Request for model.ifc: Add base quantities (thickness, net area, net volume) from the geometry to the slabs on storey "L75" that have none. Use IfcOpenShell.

First a look at what the model holds.

```python
import ifcopenshell
import ifcopenshell.util.element
import ifcopenshell.util.unit

model = ifcopenshell.open("model.ifc")
print(model.schema)
for unit_type in ("LENGTHUNIT", "AREAUNIT", "VOLUMEUNIT"):
    print(unit_type, ifcopenshell.util.unit.calculate_unit_scale(model, unit_type))
storey = next(s for s in model.by_type("IfcBuildingStorey") if s.Name == "L75")
slabs = [e for e in ifcopenshell.util.element.get_decomposition(storey) if e.is_a("IfcSlab")]
for e in sorted(slabs, key=lambda e: e.id()):
    print(e.id(), e.is_a(), e.Name, list(ifcopenshell.util.element.get_psets(e, qtos_only=True)), sep=" | ")
```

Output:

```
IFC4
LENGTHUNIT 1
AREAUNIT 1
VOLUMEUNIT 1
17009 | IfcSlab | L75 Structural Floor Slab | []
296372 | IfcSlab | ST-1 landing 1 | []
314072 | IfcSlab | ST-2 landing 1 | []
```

```python
import ifcopenshell
import ifcopenshell.api.pset
import ifcopenshell.geom
import ifcopenshell.util.element
import ifcopenshell.util.shape
import ifcopenshell.util.unit

model = ifcopenshell.open("model.ifc")
unit_scale = ifcopenshell.util.unit.calculate_unit_scale(model)
area_scale = ifcopenshell.util.unit.calculate_unit_scale(model, "AREAUNIT")
volume_scale = ifcopenshell.util.unit.calculate_unit_scale(model, "VOLUMEUNIT")
settings = ifcopenshell.geom.settings()

storey = next(s for s in model.by_type("IfcBuildingStorey") if s.Name == "L75")
slabs = [e for e in ifcopenshell.util.element.get_decomposition(storey) if e.is_a("IfcSlab")]

for e in sorted(slabs, key=lambda e: e.id()):
    if ifcopenshell.util.element.get_psets(e, qtos_only=True, should_inherit=False):
        continue
    # Geometry comes back in metres, in the element's own axes.
    shape = ifcopenshell.geom.create_shape(settings, e)
    values = {
        "Width": ifcopenshell.util.shape.get_z(shape.geometry) / unit_scale,
        "NetArea": ifcopenshell.util.shape.get_footprint_area(shape.geometry) / area_scale,
        "NetVolume": ifcopenshell.util.shape.get_volume(shape.geometry) / volume_scale,
    }
    qto = ifcopenshell.api.pset.add_qto(model, product=e, name="Qto_SlabBaseQuantities")
    ifcopenshell.api.pset.edit_qto(model, qto=qto, properties=values)
    print(e.id(), {k: round(v, 3) for k, v in values.items()})

model.write("model-out.ifc")
```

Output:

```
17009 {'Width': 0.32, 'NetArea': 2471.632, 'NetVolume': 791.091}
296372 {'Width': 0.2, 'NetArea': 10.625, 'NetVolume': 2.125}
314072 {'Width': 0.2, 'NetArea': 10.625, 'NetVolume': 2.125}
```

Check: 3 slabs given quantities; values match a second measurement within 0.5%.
